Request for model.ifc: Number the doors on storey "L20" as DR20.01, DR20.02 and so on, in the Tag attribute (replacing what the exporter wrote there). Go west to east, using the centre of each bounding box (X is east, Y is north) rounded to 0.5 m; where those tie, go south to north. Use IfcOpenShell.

First a look at what the model holds.

```python
import ifcopenshell
import ifcopenshell.util.element
import ifcopenshell.util.placement

model = ifcopenshell.open("model.ifc")
print(model.schema)
storey = next(s for s in model.by_type("IfcBuildingStorey") if s.Name == "L20")
doors = [e for e in ifcopenshell.util.element.get_decomposition(storey) if e.is_a("IfcDoor")]
for e in sorted(doors, key=lambda e: e.id()):
    origin = ifcopenshell.util.placement.get_local_placement(e.ObjectPlacement)[:3, 3]
    print(e.id(), e.Tag, e.Name, origin.round(2) + 0.0, sep=" | ")
```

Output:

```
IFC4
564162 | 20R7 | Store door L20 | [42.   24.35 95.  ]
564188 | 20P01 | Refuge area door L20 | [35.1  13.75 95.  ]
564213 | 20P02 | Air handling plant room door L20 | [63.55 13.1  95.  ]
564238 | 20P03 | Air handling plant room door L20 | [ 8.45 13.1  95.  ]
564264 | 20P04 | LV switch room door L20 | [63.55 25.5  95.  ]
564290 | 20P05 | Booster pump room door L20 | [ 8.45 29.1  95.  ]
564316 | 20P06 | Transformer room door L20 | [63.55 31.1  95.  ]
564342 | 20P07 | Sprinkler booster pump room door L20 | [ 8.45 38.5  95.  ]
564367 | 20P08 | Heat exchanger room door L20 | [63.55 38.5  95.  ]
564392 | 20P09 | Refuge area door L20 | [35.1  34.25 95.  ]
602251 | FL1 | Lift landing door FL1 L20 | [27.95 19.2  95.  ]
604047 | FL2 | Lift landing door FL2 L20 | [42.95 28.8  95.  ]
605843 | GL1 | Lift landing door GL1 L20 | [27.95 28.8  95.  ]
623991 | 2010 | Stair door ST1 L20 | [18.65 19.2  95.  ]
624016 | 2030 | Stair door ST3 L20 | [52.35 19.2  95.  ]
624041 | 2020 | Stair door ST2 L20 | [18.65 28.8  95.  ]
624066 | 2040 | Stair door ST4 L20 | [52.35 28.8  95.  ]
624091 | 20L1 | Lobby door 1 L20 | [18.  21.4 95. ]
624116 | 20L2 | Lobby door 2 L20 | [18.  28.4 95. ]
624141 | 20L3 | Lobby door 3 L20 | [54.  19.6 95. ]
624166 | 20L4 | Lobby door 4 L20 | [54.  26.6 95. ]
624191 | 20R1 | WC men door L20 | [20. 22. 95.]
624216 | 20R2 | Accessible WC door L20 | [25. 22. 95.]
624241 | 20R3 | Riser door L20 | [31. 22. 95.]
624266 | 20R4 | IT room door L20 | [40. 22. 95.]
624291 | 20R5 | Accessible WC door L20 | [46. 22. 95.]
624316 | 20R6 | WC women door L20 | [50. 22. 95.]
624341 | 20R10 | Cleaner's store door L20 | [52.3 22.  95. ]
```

```python
import ifcopenshell
import ifcopenshell.geom
import ifcopenshell.util.element
import ifcopenshell.util.shape

model = ifcopenshell.open("model.ifc")
settings = ifcopenshell.geom.settings()
settings.set("use-world-coords", True)


def centre(element):
    shape = ifcopenshell.geom.create_shape(settings, element)
    return ifcopenshell.util.shape.get_bbox_centroid(shape.geometry)


storey = next(s for s in model.by_type("IfcBuildingStorey") if s.Name == "L20")
doors = [e for e in ifcopenshell.util.element.get_decomposition(storey) if e.is_a("IfcDoor")]

# Insertion points can sit at a corner or the storey origin, so sort by the geometry (in metres).
centres = {e: centre(e) for e in doors}
doors.sort(key=lambda e: (round(centres[e][0] / 0.5), centres[e][1]))

for i, e in enumerate(doors, start=1):
    number = f"DR20.{i:02d}"
    e.Tag = number
    print(e.id(), number)

model.write("model-out.ifc")
```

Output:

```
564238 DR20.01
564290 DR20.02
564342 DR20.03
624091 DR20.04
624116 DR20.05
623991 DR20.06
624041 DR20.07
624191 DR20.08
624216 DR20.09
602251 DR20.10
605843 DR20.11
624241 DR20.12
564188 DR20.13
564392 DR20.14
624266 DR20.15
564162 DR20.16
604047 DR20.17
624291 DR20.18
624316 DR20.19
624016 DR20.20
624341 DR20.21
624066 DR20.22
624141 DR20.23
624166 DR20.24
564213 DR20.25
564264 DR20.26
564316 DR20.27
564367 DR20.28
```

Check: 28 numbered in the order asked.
